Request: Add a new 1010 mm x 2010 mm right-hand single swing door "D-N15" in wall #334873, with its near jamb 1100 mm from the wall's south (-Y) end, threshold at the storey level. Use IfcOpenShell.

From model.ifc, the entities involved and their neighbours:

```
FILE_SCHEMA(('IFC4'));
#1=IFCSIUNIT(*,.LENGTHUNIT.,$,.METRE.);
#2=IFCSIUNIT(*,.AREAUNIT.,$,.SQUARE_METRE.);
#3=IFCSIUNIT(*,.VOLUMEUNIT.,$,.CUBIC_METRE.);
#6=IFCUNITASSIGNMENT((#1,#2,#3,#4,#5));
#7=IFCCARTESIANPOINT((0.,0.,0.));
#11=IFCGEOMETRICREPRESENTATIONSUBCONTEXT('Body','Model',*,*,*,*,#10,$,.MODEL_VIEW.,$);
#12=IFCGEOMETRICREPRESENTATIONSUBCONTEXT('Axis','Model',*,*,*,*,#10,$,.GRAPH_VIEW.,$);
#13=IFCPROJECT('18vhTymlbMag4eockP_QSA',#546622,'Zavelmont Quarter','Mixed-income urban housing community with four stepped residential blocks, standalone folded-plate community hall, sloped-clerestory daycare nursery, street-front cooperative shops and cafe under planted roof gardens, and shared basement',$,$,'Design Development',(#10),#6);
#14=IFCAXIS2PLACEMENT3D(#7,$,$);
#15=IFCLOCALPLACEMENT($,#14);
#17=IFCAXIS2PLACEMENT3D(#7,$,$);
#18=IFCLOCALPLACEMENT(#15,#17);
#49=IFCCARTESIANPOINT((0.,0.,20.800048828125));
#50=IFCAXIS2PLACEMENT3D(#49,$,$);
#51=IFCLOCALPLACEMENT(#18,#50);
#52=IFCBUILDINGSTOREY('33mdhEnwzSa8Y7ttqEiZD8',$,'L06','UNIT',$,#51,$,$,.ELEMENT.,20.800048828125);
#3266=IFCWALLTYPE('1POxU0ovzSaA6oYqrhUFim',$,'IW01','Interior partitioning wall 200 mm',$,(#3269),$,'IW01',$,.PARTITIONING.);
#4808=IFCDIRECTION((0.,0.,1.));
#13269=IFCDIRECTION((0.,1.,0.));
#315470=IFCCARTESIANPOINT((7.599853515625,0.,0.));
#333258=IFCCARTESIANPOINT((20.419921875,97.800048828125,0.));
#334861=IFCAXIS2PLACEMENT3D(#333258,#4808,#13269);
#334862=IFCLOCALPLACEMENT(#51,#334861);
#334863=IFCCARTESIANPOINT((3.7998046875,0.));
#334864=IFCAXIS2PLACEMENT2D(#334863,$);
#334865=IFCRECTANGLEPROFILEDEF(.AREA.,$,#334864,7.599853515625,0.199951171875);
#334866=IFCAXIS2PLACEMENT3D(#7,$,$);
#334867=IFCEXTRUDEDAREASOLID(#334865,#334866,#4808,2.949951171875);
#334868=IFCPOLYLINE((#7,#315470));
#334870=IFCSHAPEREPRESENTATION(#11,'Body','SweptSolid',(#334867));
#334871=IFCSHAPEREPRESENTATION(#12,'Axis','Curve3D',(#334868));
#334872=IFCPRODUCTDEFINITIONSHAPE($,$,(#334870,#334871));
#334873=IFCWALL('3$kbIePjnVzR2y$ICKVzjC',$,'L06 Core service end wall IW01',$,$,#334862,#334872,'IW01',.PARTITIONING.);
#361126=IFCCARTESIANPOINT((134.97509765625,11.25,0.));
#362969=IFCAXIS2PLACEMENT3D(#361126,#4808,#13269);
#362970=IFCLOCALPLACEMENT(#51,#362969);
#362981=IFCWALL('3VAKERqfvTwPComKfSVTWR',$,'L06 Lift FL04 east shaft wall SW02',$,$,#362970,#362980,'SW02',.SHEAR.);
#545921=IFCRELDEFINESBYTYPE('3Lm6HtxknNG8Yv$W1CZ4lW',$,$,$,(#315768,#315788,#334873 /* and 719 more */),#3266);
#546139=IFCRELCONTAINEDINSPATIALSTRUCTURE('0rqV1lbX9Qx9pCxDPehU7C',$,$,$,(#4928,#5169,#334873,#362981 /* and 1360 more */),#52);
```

```python
import numpy as np
import ifcopenshell
import ifcopenshell.api.feature
import ifcopenshell.api.geometry
import ifcopenshell.api.root
import ifcopenshell.api.spatial
import ifcopenshell.geom
import ifcopenshell.util.element
import ifcopenshell.util.placement
import ifcopenshell.util.representation
import ifcopenshell.util.shape
import ifcopenshell.util.unit

model = ifcopenshell.open("model.ifc")
unit_scale = ifcopenshell.util.unit.calculate_unit_scale(model)
settings = ifcopenshell.geom.settings()


def volume(element):
    """Net volume in cubic metres, openings subtracted."""
    shape = ifcopenshell.geom.create_shape(settings, element)
    return ifcopenshell.util.shape.get_volume(shape.geometry)


wall = model.by_guid("3$kbIePjnVzR2y$ICKVzjC")
storey = ifcopenshell.util.element.get_container(wall, ifc_class="IfcBuildingStorey")
context = ifcopenshell.util.representation.get_context(model, "Model", "Body", "MODEL_VIEW")
before = volume(wall)

width, height, from_end, sill = 1.01, 2.01, 1.1, 0.0  # metres

# The wall runs along its own X axis, and the end named is its -X end.
wall_shape = ifcopenshell.geom.create_shape(settings, wall)
x, y, z = ifcopenshell.util.shape.get_vertices(wall_shape.geometry).T
start = x.min() + from_end
face, thickness = float(y.min()), float(y.max() - y.min())
wall_matrix = ifcopenshell.util.placement.get_local_placement(wall.ObjectPlacement)
level = ifcopenshell.util.placement.get_local_placement(storey.ObjectPlacement)[2, 3]


def in_wall(x, y):
    """Placement at x, y metres in the wall's axes, at sill height."""
    matrix = wall_matrix.copy()
    matrix[:, 3] = wall_matrix @ np.array([x / unit_scale, y / unit_scale, 0.0, 1.0])
    matrix[2, 3] = level + sill / unit_scale
    return matrix


# Opening: a box that overshoots both wall faces by 50 mm.
opening = ifcopenshell.api.root.create_entity(model, ifc_class="IfcOpeningElement", predefined_type="OPENING")
box = ifcopenshell.api.geometry.add_wall_representation(
    model, context=context, length=width, height=height, thickness=thickness + 0.1
)
ifcopenshell.api.geometry.assign_representation(model, product=opening, representation=box)
ifcopenshell.api.geometry.edit_object_placement(model, product=opening, matrix=in_wall(start, face - 0.05), is_si=False)
ifcopenshell.api.feature.add_feature(model, feature=opening, element=wall)

door = ifcopenshell.api.root.create_entity(model, ifc_class="IfcDoor", name="D-N15", predefined_type="DOOR")
door.OverallWidth, door.OverallHeight = width / unit_scale, height / unit_scale
door.OperationType = "SINGLE_SWING_RIGHT"
body = ifcopenshell.api.geometry.add_door_representation(
    model,
    context=context,
    overall_width=door.OverallWidth,
    overall_height=door.OverallHeight,
    operation_type="SINGLE_SWING_RIGHT",
    lining_properties={"LiningDepth": thickness / unit_scale, "ThresholdDepth": thickness / unit_scale},
)
ifcopenshell.api.geometry.assign_representation(model, product=door, representation=body)
ifcopenshell.api.spatial.assign_container(model, products=[door], relating_structure=storey)
ifcopenshell.api.feature.add_filling(model, opening=opening, element=door)

# The lining spans the wall, so the door starts at the wall face.
ifcopenshell.api.geometry.edit_object_placement(model, product=door, matrix=in_wall(start, face), is_si=False)

after = volume(wall)

print(f"wall volume {before:.3f} -> {after:.3f} m3")

model.write("model_edited.ifc")
```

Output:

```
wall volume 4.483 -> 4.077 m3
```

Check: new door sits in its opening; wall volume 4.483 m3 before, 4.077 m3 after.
